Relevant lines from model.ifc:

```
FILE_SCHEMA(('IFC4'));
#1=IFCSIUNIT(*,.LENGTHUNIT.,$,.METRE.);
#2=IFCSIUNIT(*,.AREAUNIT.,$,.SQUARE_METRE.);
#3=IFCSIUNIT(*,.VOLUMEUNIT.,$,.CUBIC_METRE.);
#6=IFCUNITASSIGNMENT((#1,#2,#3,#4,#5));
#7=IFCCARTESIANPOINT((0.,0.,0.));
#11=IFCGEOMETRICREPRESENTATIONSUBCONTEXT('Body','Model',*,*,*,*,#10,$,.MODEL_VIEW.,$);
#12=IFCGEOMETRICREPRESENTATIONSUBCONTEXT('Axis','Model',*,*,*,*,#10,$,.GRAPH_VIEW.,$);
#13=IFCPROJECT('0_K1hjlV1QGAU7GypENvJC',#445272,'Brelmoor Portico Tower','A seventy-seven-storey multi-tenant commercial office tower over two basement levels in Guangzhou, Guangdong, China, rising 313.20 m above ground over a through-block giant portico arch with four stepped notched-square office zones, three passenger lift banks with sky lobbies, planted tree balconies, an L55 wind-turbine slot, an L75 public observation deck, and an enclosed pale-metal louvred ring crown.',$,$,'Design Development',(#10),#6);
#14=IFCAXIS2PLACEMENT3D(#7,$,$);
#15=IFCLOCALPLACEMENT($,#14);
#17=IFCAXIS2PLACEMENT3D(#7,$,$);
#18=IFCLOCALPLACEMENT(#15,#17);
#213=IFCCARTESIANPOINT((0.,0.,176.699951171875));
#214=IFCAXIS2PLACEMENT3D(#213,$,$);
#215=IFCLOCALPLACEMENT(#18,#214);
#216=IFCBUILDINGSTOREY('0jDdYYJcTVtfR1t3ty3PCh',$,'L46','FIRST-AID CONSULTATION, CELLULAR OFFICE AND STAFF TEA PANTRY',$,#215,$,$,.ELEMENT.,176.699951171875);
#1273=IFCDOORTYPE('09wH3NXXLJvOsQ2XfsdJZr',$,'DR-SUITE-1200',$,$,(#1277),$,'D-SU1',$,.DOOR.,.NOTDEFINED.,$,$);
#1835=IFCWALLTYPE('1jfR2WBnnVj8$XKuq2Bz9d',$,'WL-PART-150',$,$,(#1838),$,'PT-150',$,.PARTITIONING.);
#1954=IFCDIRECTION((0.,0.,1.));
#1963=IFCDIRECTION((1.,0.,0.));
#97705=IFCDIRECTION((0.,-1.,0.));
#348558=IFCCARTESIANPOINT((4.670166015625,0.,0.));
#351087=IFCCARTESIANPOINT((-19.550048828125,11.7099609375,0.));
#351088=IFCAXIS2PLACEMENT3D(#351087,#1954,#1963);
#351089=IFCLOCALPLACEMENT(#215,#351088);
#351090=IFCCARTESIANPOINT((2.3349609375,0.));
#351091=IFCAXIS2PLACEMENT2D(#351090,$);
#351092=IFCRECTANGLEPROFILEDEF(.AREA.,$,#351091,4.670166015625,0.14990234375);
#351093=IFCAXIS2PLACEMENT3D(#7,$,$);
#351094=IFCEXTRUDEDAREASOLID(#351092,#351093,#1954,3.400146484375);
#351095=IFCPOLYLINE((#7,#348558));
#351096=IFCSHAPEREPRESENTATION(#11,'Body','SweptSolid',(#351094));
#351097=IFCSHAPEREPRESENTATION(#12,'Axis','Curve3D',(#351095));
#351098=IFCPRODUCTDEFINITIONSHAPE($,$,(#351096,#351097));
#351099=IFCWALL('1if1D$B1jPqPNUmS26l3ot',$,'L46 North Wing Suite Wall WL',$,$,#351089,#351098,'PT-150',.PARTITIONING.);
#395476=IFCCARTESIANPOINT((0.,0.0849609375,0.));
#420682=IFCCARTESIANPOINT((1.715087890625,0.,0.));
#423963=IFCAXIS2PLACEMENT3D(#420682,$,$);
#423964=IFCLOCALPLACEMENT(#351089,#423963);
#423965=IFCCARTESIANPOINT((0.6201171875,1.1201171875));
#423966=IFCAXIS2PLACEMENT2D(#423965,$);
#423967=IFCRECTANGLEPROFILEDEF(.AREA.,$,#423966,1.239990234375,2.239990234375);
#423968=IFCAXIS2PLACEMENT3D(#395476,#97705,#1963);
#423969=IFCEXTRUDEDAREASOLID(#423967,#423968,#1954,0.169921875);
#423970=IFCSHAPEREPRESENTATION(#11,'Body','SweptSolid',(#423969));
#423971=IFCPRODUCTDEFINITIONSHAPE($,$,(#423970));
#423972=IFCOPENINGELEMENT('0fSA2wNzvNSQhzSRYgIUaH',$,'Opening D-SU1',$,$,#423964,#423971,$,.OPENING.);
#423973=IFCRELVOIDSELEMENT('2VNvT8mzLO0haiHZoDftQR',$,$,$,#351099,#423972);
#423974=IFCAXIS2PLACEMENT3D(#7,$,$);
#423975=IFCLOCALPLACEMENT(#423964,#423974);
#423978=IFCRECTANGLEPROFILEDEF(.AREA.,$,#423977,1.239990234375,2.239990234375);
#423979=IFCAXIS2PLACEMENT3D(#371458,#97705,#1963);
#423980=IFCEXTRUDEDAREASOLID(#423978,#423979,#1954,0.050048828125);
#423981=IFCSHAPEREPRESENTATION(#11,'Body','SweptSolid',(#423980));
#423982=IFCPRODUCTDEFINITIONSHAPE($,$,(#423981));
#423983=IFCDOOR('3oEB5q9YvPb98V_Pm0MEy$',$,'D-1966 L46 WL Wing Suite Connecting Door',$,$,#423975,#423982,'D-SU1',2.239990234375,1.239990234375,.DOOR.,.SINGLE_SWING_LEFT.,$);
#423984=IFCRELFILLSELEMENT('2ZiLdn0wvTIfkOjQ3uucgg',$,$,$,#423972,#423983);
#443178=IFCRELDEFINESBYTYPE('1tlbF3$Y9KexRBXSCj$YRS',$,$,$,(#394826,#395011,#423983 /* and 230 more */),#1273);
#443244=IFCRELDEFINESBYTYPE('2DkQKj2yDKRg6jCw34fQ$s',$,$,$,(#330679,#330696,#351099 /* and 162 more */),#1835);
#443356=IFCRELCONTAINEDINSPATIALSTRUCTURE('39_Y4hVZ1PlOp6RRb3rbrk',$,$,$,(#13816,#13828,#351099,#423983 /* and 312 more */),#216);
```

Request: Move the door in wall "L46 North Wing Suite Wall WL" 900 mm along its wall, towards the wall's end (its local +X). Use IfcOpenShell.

```python
import ifcopenshell
import ifcopenshell.api.geometry
import ifcopenshell.util.placement

model = ifcopenshell.open("model.ifc")

door = model.by_guid("3oEB5q9YvPb98V_Pm0MEy$")
opening = door.FillsVoids[0].RelatingOpeningElement
wall = opening.VoidsElements[0].RelatingBuildingElement

wall_matrix = ifcopenshell.util.placement.get_local_placement(wall.ObjectPlacement)
shift = wall_matrix[:3, 0] * 0.9
before = ifcopenshell.util.placement.get_local_placement(door.ObjectPlacement)[:3, 3].copy()

# The door is placed relative to its opening, so it follows when the opening moves.
matrix = ifcopenshell.util.placement.get_local_placement(opening.ObjectPlacement)
matrix[:3, 3] += shift
ifcopenshell.api.geometry.edit_object_placement(
    model, product=opening, matrix=matrix, is_si=False, should_transform_children=True
)

after = ifcopenshell.util.placement.get_local_placement(door.ObjectPlacement)[:3, 3]
print("door moved by", (after - before).round(3) + 0.0)

model.write("model_updated.ifc")
```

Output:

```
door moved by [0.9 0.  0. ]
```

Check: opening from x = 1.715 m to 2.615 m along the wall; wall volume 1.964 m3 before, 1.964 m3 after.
